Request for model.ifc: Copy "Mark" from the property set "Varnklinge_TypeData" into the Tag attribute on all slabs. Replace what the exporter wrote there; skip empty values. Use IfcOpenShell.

First a look at what the model holds.

```python
import ifcopenshell
import ifcopenshell.util.element

model = ifcopenshell.open("model.ifc")
print(model.schema)
slabs = model.by_type("IfcSlab")
print(len(slabs), "slabs")
for e in slabs[:8]:
    source = ifcopenshell.util.element.get_pset(e, "Varnklinge_TypeData", "Mark")
    target = e.Tag
    print(e.id(), repr(source), repr(target), sep=" | ")
```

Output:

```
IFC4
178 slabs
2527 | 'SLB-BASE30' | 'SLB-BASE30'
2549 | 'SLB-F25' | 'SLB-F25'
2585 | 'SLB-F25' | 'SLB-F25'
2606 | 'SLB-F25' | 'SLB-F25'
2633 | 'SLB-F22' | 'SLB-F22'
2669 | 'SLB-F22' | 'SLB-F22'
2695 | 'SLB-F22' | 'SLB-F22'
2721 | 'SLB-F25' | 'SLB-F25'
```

```python
import ifcopenshell
import ifcopenshell.util.element

model = ifcopenshell.open("model.ifc")

count = 0
for e in model.by_type("IfcSlab"):
    value = ifcopenshell.util.element.get_pset(e, "Varnklinge_TypeData", "Mark")
    current = e.Tag
    if not value or not value.strip() or current == value:
        continue
    e.Tag = value
    count += 1

print(count, "slabs updated")

model.write("model_v2.ifc")
```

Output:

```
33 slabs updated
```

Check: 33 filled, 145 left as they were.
